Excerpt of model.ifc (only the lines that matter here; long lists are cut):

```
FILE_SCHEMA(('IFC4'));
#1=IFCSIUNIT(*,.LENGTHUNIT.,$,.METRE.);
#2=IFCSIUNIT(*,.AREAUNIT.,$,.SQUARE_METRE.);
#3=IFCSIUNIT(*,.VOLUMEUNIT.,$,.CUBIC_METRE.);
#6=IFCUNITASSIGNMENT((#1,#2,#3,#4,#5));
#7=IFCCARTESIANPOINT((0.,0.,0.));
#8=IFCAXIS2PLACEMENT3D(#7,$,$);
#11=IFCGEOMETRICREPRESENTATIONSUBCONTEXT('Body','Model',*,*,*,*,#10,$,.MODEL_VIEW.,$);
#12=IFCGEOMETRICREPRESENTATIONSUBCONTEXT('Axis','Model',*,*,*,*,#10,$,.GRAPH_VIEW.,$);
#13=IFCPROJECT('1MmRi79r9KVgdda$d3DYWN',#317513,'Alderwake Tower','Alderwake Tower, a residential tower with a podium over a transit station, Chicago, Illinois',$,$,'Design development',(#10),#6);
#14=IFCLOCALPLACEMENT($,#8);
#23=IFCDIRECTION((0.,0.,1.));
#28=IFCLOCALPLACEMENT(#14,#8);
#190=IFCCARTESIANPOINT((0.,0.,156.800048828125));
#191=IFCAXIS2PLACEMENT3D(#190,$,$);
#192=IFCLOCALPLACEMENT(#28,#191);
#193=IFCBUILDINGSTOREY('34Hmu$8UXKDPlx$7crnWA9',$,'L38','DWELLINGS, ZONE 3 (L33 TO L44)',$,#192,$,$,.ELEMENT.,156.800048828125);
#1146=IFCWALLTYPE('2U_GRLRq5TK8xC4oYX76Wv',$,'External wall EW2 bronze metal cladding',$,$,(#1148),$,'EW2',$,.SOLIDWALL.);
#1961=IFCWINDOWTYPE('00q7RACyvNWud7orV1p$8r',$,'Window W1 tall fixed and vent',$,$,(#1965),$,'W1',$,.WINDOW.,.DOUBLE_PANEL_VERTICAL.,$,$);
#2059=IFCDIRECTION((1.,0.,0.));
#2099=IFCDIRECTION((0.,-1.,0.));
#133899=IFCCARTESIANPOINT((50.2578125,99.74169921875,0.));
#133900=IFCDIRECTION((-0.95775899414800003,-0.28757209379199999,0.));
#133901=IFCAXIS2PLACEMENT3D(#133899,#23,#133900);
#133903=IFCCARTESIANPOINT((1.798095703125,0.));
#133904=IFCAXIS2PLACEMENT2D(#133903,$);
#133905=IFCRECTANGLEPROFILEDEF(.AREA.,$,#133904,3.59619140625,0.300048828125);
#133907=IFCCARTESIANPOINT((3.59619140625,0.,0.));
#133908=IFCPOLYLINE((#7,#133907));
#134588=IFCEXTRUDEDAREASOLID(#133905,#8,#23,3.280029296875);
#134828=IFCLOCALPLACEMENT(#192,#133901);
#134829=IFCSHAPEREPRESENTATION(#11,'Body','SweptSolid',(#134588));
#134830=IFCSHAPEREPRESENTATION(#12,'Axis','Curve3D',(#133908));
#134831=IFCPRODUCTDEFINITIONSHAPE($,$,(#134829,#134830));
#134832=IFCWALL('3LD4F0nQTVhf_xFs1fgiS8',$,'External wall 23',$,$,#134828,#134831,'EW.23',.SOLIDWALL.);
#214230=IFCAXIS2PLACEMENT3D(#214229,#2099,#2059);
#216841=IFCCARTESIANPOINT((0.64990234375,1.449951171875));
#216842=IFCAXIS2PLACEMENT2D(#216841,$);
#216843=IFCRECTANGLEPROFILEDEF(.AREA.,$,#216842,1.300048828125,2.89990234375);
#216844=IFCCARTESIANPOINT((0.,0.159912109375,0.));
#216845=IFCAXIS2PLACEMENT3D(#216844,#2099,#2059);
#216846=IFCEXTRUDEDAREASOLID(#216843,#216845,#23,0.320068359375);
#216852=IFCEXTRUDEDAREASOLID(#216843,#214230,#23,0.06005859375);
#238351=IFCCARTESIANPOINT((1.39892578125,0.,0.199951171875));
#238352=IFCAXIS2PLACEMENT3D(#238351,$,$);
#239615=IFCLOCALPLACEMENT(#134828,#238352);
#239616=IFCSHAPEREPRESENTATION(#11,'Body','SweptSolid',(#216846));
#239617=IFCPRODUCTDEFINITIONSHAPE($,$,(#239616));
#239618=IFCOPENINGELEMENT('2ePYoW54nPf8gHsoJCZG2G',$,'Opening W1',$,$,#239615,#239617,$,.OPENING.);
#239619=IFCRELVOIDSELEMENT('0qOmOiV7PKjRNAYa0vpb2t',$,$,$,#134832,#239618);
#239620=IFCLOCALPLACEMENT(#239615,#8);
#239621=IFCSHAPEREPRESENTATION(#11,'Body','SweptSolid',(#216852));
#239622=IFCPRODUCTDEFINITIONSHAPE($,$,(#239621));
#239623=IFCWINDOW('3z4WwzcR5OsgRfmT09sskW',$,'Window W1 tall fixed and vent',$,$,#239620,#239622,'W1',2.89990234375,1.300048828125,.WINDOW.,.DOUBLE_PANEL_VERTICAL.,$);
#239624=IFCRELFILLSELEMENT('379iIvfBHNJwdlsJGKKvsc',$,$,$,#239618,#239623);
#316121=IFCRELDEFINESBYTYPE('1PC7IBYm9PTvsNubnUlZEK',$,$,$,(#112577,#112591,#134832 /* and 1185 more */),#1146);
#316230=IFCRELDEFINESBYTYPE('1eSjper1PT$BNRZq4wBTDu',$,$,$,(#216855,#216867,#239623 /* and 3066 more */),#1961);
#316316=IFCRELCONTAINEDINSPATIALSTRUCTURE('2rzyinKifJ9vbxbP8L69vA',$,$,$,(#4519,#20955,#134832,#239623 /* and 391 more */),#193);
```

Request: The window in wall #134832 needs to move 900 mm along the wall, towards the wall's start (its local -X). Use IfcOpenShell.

```python
import ifcopenshell
import ifcopenshell.api.geometry
import ifcopenshell.util.placement
import ifcopenshell.util.unit

model = ifcopenshell.open("model.ifc")
unit_scale = ifcopenshell.util.unit.calculate_unit_scale(model)

window = model.by_guid("3z4WwzcR5OsgRfmT09sskW")
opening = window.FillsVoids[0].RelatingOpeningElement
wall = opening.VoidsElements[0].RelatingBuildingElement

wall_matrix = ifcopenshell.util.placement.get_local_placement(wall.ObjectPlacement)
shift = wall_matrix[:3, 0] * -0.9 / unit_scale
before = ifcopenshell.util.placement.get_local_placement(window.ObjectPlacement)[:3, 3].copy()

# The window is placed relative to its opening, so it follows when the opening moves.
matrix = ifcopenshell.util.placement.get_local_placement(opening.ObjectPlacement)
matrix[:3, 3] += shift
ifcopenshell.api.geometry.edit_object_placement(
    model, product=opening, matrix=matrix, is_si=False, should_transform_children=True
)

after = ifcopenshell.util.placement.get_local_placement(window.ObjectPlacement)[:3, 3]
print("window moved by", (after - before).round(3) + 0.0)

model.write("model_updated.ifc")
```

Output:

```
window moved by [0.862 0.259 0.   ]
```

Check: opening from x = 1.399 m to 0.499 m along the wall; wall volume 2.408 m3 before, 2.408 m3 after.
